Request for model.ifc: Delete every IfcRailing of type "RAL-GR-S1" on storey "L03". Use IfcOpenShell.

First a look at what the model holds.

```python
import ifcopenshell
import ifcopenshell.util.element

model = ifcopenshell.open("model.ifc")
print(model.schema)
storey = next(s for s in model.by_type("IfcBuildingStorey") if s.Name == "L03")
railings = [e for e in ifcopenshell.util.element.get_decomposition(storey) if e.is_a("IfcRailing")]
seen = {}
for e in railings:
    element_type = ifcopenshell.util.element.get_type(e)
    name = element_type.Name if element_type not in (None, e) else None
    seen[name] = seen.get(name, 0) + 1
for name, count in sorted(seen.items(), key=str):
    print(count, "x", name)
```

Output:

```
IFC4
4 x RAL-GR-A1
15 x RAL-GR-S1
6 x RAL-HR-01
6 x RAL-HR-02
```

```python
import ifcopenshell
import ifcopenshell.api.root
import ifcopenshell.util.element

model = ifcopenshell.open("model.ifc")

storey = next(s for s in model.by_type("IfcBuildingStorey") if s.Name == "L03")
railings = [e for e in ifcopenshell.util.element.get_decomposition(storey) if e.is_a("IfcRailing")]
targets = [e for e in railings if (t := ifcopenshell.util.element.get_type(e)) not in (None, e) and t.Name == "RAL-GR-S1"]

for e in targets:
    ifcopenshell.api.root.remove_product(model, product=e)
print(len(targets), "removed")

model.write("model_rev.ifc")
```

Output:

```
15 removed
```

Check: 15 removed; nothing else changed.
